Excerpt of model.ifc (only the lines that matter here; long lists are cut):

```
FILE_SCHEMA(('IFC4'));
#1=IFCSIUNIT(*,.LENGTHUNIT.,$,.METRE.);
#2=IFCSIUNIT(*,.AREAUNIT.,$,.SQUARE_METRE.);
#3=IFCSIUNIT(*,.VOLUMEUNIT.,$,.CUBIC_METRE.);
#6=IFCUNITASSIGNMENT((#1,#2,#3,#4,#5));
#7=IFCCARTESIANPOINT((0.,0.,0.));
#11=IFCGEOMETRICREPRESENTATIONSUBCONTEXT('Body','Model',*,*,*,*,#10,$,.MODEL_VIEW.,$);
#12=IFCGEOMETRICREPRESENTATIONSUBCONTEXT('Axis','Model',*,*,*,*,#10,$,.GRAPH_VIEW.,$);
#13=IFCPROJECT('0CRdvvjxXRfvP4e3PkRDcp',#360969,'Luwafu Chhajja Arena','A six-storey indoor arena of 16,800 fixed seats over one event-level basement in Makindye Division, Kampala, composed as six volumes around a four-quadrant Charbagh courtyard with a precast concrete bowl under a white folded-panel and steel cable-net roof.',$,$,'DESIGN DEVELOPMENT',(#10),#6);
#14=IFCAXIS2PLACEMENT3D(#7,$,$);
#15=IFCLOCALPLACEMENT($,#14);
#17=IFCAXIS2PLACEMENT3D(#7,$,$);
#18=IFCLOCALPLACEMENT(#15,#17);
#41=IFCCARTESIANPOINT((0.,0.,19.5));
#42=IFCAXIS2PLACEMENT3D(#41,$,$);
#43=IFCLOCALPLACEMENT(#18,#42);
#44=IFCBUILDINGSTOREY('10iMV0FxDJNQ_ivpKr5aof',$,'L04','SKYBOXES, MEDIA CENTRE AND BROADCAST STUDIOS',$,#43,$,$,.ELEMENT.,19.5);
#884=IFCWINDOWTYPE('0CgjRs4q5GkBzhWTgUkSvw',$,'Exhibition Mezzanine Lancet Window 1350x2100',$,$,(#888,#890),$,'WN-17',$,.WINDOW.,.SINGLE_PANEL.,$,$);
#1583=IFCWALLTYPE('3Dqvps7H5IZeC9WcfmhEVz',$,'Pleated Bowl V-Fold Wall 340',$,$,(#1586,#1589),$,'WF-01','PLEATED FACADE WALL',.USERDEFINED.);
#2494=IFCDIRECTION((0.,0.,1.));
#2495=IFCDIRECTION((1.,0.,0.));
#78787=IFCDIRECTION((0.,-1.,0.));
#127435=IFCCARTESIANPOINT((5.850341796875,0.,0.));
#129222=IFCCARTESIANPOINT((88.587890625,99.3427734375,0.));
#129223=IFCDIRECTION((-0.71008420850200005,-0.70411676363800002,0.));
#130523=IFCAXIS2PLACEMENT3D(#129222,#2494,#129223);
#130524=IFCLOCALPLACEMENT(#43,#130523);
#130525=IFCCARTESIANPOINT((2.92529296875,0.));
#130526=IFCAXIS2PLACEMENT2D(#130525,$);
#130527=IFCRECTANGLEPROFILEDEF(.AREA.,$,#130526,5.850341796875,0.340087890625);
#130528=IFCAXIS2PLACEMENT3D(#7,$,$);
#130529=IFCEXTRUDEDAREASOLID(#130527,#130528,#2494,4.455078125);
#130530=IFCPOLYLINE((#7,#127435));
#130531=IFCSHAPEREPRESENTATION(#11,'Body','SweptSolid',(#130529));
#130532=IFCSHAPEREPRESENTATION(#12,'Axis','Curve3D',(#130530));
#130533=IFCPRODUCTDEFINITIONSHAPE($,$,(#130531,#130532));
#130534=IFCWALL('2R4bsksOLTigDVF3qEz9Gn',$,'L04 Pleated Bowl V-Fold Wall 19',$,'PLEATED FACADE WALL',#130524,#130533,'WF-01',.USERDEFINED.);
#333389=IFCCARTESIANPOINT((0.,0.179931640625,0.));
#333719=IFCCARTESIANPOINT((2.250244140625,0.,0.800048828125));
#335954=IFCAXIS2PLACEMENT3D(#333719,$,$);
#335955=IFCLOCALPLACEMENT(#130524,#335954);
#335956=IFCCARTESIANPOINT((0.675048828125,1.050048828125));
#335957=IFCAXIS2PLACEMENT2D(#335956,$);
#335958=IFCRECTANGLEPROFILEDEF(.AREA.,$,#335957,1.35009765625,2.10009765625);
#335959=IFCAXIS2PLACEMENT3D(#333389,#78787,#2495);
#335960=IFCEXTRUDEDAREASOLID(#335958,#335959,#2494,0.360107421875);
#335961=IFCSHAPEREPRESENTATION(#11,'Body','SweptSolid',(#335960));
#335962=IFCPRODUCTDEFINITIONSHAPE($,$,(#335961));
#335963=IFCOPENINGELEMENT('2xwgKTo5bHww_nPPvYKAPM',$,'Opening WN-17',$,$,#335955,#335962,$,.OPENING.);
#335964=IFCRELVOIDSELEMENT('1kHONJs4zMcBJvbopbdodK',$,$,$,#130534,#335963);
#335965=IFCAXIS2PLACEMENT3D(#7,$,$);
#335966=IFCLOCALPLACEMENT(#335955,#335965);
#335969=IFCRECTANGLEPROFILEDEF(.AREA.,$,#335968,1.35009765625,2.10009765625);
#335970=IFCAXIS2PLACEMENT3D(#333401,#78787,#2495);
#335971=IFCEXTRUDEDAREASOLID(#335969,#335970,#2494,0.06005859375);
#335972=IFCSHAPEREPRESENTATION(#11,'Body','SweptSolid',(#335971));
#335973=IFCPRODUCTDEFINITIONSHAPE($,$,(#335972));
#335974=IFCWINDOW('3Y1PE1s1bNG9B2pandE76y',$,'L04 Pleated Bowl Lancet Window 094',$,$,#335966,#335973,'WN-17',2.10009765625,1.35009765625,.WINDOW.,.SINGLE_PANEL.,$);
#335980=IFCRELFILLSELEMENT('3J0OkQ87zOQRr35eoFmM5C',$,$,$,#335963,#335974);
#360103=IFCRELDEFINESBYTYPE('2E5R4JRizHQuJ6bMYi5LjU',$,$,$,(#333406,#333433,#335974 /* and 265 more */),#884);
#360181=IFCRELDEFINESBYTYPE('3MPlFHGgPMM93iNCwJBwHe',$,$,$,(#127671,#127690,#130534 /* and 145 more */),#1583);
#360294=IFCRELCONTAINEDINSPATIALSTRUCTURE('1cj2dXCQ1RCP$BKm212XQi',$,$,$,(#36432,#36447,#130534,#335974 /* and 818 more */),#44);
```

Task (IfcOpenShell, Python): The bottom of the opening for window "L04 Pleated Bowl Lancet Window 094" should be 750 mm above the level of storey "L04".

```python
import numpy as np
import ifcopenshell
import ifcopenshell.api.geometry
import ifcopenshell.geom
import ifcopenshell.util.element
import ifcopenshell.util.placement
import ifcopenshell.util.shape
import ifcopenshell.util.unit

model = ifcopenshell.open("model.ifc")
unit_scale = ifcopenshell.util.unit.calculate_unit_scale(model)

window = model.by_guid("3Y1PE1s1bNG9B2pandE76y")
opening = window.FillsVoids[0].RelatingOpeningElement
storey = ifcopenshell.util.element.get_container(window, ifc_class="IfcBuildingStorey")
level = ifcopenshell.util.placement.get_local_placement(storey.ObjectPlacement)[2, 3]

# The opening's origin need not be at the sill, so measure its lowest point.
shape = ifcopenshell.geom.create_shape(ifcopenshell.geom.settings(), opening)
bottom = ifcopenshell.util.shape.get_shape_bottom_elevation(shape, shape.geometry) / unit_scale
dz = level + 0.75 / unit_scale - bottom

shift = np.array([0.0, 0.0, dz])
# The window is placed relative to its opening, so it follows when the opening moves.
matrix = ifcopenshell.util.placement.get_local_placement(opening.ObjectPlacement)
matrix[:3, 3] += shift
ifcopenshell.api.geometry.edit_object_placement(
    model, product=opening, matrix=matrix, is_si=False, should_transform_children=True
)

print(f"moved by {dz * unit_scale:+.3f} m")

model.write("model_rev.ifc")
```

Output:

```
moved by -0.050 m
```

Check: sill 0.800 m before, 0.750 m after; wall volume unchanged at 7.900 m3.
